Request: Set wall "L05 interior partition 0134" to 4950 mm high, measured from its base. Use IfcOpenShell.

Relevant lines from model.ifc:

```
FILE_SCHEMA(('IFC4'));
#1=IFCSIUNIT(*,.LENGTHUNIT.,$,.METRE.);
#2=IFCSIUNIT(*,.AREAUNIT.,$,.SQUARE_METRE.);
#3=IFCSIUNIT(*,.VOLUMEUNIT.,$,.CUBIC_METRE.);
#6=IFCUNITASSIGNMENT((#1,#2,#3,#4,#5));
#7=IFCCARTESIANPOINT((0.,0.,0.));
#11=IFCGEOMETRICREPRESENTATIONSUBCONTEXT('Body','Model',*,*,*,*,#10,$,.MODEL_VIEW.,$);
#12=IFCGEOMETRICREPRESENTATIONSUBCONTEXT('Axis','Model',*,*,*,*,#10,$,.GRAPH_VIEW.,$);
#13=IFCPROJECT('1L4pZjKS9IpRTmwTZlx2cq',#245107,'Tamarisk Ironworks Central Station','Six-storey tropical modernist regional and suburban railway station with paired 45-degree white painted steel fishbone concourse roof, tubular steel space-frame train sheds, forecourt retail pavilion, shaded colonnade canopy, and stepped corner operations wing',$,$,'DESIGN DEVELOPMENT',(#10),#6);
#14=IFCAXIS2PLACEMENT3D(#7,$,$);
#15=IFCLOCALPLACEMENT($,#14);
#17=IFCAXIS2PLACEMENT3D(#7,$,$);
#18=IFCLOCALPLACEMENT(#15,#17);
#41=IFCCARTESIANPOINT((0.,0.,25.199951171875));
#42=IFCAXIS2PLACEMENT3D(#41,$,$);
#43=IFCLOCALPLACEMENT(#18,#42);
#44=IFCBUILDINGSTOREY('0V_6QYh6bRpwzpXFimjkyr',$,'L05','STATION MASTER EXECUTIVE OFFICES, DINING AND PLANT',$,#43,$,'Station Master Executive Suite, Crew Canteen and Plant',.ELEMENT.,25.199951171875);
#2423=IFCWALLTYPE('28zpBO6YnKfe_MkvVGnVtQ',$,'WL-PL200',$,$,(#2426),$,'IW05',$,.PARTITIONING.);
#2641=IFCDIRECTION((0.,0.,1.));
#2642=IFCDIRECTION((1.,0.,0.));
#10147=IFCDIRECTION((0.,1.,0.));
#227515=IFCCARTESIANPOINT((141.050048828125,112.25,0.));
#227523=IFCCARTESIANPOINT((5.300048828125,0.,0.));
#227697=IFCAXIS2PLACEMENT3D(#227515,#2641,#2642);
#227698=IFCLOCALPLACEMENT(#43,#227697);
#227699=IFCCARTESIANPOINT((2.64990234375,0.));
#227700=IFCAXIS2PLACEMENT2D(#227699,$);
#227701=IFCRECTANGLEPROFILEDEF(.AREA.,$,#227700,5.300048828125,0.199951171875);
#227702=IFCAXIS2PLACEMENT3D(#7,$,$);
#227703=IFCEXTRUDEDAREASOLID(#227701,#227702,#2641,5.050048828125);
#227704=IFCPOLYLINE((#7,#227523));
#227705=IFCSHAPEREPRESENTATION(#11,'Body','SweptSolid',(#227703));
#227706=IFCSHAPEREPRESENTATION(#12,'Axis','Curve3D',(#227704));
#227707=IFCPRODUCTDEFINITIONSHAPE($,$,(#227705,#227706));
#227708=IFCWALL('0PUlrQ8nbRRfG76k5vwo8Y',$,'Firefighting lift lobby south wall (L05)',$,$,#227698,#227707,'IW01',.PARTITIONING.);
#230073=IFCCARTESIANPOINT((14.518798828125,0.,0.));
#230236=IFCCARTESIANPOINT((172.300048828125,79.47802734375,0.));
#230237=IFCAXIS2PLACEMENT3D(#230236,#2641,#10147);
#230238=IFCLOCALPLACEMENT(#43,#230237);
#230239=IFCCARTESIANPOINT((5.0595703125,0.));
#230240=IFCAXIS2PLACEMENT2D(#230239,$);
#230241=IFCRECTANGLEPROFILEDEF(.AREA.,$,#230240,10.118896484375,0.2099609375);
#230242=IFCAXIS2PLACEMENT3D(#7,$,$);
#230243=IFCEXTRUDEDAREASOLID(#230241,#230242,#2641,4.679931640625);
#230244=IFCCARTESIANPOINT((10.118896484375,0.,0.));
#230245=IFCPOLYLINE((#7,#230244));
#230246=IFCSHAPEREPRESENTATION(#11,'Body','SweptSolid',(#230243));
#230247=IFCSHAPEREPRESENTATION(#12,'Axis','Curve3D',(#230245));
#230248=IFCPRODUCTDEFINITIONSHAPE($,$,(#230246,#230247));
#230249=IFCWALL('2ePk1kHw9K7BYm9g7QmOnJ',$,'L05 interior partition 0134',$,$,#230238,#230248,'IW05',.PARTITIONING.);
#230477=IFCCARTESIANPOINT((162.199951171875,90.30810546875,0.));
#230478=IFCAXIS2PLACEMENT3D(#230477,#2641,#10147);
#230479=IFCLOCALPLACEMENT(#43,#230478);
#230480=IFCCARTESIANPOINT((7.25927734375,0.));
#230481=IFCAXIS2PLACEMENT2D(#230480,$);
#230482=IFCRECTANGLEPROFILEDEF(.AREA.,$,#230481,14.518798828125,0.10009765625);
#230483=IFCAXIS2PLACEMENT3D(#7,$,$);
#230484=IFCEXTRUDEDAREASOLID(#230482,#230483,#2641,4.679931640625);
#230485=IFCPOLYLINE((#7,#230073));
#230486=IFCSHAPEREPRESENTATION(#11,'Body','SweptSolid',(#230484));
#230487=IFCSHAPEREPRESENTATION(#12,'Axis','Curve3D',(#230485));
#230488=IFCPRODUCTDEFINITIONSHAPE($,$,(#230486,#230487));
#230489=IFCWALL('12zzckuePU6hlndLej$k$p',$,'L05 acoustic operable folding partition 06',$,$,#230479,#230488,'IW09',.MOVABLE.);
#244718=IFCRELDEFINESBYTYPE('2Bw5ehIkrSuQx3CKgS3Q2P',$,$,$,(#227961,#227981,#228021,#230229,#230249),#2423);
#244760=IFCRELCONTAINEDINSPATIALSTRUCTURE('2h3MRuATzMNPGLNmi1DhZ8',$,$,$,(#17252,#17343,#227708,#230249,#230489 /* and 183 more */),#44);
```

```python
import ifcopenshell
import ifcopenshell.geom
import ifcopenshell.util.representation
import ifcopenshell.util.shape

model = ifcopenshell.open("model.ifc")
settings = ifcopenshell.geom.settings()


def volume(element):
    """Net volume in cubic metres, openings subtracted."""
    shape = ifcopenshell.geom.create_shape(settings, element)
    return ifcopenshell.util.shape.get_volume(shape.geometry)


wall = model.by_id(230249)
before = volume(wall)

body = ifcopenshell.util.representation.get_representation(wall, "Model", "Body")
solid = body.Items[0]
old_height = solid.Depth
solid.Depth = 4.95
after = volume(wall)

print(f"height {old_height:g} -> {solid.Depth:g}, volume {before:.3f} -> {after:.3f} m3")

model.write("model_updated.ifc")
```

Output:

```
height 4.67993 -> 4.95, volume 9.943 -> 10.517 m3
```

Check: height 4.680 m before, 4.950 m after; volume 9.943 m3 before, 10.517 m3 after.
